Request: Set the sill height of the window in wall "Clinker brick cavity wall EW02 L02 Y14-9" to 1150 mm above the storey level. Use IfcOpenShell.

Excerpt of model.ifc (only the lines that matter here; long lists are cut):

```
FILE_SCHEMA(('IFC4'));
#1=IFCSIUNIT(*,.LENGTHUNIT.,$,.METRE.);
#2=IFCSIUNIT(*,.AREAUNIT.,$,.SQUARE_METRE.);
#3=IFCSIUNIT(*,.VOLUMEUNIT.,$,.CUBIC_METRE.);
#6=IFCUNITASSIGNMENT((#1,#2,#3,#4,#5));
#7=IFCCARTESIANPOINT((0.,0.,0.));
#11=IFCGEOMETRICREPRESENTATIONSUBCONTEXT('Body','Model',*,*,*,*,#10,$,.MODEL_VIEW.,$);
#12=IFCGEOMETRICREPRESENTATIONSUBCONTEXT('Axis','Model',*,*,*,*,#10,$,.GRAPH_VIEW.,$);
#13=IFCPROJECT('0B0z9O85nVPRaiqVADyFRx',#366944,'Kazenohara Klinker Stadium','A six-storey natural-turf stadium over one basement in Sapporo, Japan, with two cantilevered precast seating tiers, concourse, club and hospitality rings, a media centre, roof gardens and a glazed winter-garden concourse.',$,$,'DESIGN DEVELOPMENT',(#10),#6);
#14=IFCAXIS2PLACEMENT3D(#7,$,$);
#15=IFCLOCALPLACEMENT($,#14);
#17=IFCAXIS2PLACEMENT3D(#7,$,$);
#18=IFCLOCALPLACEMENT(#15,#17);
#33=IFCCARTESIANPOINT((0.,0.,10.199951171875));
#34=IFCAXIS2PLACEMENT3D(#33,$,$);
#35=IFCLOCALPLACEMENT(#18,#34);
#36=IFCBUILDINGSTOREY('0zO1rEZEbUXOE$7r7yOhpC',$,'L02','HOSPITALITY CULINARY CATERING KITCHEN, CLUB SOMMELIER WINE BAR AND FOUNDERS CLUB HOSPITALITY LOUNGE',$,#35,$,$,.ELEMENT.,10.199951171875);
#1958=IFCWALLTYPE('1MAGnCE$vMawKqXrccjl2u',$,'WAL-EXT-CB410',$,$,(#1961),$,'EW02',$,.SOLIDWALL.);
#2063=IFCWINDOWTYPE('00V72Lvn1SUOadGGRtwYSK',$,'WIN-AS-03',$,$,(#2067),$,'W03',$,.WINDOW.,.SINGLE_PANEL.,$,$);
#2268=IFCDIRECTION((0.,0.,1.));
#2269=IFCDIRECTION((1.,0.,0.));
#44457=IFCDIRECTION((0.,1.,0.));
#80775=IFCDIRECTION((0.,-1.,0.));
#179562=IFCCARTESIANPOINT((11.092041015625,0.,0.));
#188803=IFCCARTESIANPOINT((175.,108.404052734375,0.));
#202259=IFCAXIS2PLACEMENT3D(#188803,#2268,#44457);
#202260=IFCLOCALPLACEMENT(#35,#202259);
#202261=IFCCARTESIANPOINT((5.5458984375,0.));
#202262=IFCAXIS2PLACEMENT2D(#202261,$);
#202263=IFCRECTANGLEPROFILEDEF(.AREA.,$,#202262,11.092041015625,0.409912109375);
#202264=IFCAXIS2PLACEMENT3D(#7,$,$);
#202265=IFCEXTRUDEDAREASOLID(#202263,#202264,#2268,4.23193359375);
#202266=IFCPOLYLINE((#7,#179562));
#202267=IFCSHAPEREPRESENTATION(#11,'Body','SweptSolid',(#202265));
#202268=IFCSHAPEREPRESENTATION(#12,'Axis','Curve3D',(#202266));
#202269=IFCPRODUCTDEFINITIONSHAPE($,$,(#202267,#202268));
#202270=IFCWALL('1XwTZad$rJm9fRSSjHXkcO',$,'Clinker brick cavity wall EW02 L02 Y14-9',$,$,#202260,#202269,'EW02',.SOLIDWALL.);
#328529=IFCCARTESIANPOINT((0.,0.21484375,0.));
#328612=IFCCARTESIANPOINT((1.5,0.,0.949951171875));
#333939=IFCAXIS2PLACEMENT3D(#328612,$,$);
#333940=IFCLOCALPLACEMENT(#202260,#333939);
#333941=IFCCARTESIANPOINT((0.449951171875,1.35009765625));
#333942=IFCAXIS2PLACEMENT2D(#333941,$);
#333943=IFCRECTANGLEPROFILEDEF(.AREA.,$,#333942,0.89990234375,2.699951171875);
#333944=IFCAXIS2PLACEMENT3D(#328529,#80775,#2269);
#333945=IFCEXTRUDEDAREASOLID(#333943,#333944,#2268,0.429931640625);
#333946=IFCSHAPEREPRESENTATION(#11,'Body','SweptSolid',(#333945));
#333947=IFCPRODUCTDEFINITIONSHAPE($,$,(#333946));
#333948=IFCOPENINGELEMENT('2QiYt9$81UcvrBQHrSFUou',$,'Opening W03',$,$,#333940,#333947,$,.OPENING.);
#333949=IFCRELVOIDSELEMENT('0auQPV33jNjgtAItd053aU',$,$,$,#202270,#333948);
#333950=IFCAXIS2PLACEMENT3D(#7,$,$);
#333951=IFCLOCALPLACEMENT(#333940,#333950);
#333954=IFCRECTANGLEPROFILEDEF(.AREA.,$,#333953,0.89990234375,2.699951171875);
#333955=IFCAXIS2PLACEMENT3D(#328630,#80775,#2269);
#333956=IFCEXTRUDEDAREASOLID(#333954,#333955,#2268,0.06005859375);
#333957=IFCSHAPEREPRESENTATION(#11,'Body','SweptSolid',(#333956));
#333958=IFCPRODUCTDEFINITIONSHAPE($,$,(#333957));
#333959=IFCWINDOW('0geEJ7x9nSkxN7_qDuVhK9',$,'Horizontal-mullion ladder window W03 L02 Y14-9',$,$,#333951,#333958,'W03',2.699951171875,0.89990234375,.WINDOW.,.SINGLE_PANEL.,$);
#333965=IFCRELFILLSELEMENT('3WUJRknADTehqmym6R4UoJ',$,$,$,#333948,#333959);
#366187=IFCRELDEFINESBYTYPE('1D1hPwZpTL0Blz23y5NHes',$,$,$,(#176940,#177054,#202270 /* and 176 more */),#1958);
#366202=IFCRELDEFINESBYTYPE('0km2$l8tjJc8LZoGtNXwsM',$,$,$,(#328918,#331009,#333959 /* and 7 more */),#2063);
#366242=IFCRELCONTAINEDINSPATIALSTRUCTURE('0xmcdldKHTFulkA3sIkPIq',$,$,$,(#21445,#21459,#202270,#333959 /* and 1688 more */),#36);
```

```python
import numpy as np
import ifcopenshell
import ifcopenshell.api.geometry
import ifcopenshell.geom
import ifcopenshell.util.element
import ifcopenshell.util.placement
import ifcopenshell.util.shape
import ifcopenshell.util.unit

model = ifcopenshell.open("model.ifc")
unit_scale = ifcopenshell.util.unit.calculate_unit_scale(model)

window = model.by_guid("0geEJ7x9nSkxN7_qDuVhK9")
opening = window.FillsVoids[0].RelatingOpeningElement
storey = ifcopenshell.util.element.get_container(window, ifc_class="IfcBuildingStorey")
level = ifcopenshell.util.placement.get_local_placement(storey.ObjectPlacement)[2, 3]

# The opening's origin need not be at the sill, so measure its lowest point.
shape = ifcopenshell.geom.create_shape(ifcopenshell.geom.settings(), opening)
bottom = ifcopenshell.util.shape.get_shape_bottom_elevation(shape, shape.geometry) / unit_scale
dz = level + 1.15 - bottom

shift = np.array([0.0, 0.0, dz])
# The window is placed relative to its opening, so it follows when the opening moves.
matrix = ifcopenshell.util.placement.get_local_placement(opening.ObjectPlacement)
matrix[:3, 3] += shift
ifcopenshell.api.geometry.edit_object_placement(
    model, product=opening, matrix=matrix, is_si=False, should_transform_children=True
)

print(f"moved by {dz * unit_scale:+.3f} m")

model.write("model-out.ifc")
```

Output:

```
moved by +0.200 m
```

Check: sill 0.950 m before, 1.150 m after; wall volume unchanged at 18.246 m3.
